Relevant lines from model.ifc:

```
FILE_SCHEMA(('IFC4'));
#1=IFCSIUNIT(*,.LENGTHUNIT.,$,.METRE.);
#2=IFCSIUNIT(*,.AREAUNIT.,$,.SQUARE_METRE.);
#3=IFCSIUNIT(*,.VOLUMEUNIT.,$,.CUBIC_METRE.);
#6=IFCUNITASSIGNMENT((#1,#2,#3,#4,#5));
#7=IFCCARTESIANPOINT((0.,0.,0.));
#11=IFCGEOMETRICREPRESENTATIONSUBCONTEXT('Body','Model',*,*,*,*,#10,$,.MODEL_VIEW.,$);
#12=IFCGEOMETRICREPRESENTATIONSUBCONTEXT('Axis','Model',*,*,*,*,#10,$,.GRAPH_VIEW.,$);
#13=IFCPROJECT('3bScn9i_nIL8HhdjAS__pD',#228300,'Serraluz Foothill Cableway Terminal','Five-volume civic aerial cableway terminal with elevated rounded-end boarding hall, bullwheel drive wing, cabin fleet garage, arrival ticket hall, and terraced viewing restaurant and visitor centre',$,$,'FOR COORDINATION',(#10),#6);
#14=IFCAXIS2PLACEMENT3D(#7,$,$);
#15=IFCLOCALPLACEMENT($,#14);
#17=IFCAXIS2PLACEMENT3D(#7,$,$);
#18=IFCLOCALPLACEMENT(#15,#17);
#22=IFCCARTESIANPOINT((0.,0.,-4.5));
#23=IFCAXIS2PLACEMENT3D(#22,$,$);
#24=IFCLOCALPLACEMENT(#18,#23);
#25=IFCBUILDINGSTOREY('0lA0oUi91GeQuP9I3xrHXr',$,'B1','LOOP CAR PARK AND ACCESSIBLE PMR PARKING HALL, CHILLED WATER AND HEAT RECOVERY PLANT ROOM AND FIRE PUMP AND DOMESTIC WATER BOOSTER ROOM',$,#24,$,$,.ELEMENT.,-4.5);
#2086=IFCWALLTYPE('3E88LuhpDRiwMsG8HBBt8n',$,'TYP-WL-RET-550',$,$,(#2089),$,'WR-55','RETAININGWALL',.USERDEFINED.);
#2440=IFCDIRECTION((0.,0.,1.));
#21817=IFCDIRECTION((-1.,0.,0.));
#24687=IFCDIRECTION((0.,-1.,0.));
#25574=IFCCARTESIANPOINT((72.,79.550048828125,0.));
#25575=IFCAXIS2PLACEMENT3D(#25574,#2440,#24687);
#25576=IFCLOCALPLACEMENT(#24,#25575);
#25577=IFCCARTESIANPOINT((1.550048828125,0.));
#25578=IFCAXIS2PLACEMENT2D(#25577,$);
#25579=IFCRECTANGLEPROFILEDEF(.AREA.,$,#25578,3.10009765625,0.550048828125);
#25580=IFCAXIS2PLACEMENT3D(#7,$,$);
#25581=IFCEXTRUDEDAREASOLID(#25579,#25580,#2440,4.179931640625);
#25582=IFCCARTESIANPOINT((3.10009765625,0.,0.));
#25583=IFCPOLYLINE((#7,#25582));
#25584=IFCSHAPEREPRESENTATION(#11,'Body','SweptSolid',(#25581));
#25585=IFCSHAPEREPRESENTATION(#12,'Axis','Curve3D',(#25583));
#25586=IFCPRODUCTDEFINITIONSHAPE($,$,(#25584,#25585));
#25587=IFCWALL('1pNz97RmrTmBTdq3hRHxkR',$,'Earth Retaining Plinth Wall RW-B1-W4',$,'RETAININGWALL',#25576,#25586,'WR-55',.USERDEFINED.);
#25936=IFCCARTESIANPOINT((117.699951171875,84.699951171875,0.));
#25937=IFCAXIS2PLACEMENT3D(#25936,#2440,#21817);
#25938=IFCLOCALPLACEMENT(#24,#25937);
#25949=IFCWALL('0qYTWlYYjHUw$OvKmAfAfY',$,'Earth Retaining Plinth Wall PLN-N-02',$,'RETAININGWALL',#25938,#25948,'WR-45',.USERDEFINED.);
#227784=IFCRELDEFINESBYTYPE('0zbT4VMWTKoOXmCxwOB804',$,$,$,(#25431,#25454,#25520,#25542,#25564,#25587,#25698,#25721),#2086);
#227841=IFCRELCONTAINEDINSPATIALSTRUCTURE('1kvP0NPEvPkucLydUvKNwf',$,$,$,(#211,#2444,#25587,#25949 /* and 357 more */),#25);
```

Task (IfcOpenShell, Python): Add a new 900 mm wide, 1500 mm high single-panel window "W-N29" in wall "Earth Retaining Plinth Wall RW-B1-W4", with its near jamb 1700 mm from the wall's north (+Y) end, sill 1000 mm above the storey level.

```python
import numpy as np
import ifcopenshell
import ifcopenshell.api.feature
import ifcopenshell.api.geometry
import ifcopenshell.api.root
import ifcopenshell.api.spatial
import ifcopenshell.geom
import ifcopenshell.util.element
import ifcopenshell.util.placement
import ifcopenshell.util.representation
import ifcopenshell.util.shape
import ifcopenshell.util.unit

model = ifcopenshell.open("model.ifc")
unit_scale = ifcopenshell.util.unit.calculate_unit_scale(model)
settings = ifcopenshell.geom.settings()


def volume(element):
    """Net volume in cubic metres, openings subtracted."""
    shape = ifcopenshell.geom.create_shape(settings, element)
    return ifcopenshell.util.shape.get_volume(shape.geometry)


wall = model.by_id(25587)
storey = ifcopenshell.util.element.get_container(wall, ifc_class="IfcBuildingStorey")
context = ifcopenshell.util.representation.get_context(model, "Model", "Body", "MODEL_VIEW")
before = volume(wall)

width, height, from_end, sill = 0.9, 1.5, 1.7, 1  # metres

# The wall runs along its own X axis, and the end named is its -X end.
wall_shape = ifcopenshell.geom.create_shape(settings, wall)
x, y, z = ifcopenshell.util.shape.get_vertices(wall_shape.geometry).T
start = x.min() + from_end
face, thickness = float(y.min()), float(y.max() - y.min())
wall_matrix = ifcopenshell.util.placement.get_local_placement(wall.ObjectPlacement)
level = ifcopenshell.util.placement.get_local_placement(storey.ObjectPlacement)[2, 3]


def in_wall(x, y):
    """Placement at x, y metres in the wall's axes, at sill height."""
    matrix = wall_matrix.copy()
    matrix[:, 3] = wall_matrix @ np.array([x / unit_scale, y / unit_scale, 0.0, 1.0])
    matrix[2, 3] = level + sill / unit_scale
    return matrix


# Opening: a box that overshoots both wall faces by 50 mm.
opening = ifcopenshell.api.root.create_entity(model, ifc_class="IfcOpeningElement", predefined_type="OPENING")
box = ifcopenshell.api.geometry.add_wall_representation(
    model, context=context, length=width, height=height, thickness=thickness + 0.1
)
ifcopenshell.api.geometry.assign_representation(model, product=opening, representation=box)
ifcopenshell.api.geometry.edit_object_placement(model, product=opening, matrix=in_wall(start, face - 0.05), is_si=False)
ifcopenshell.api.feature.add_feature(model, feature=opening, element=wall)

window = ifcopenshell.api.root.create_entity(model, ifc_class="IfcWindow", name="W-N29", predefined_type="WINDOW")
window.OverallWidth, window.OverallHeight = width / unit_scale, height / unit_scale
window.PartitioningType = "SINGLE_PANEL"
body = ifcopenshell.api.geometry.add_window_representation(
    model,
    context=context,
    overall_width=window.OverallWidth,
    overall_height=window.OverallHeight,
    partition_type="SINGLE_PANEL",
)
ifcopenshell.api.geometry.assign_representation(model, product=window, representation=body)
ifcopenshell.api.spatial.assign_container(model, products=[window], relating_structure=storey)
ifcopenshell.api.feature.add_filling(model, opening=opening, element=window)

# Centre the window in the wall's thickness.
ifcopenshell.api.geometry.edit_object_placement(model, product=window, matrix=in_wall(start, face), is_si=False)
window_shape = ifcopenshell.geom.create_shape(settings, window)
depth = ifcopenshell.util.shape.get_vertices(window_shape.geometry)[:, 1]
offset = face + thickness / 2 - (depth.min() + depth.max()) / 2
ifcopenshell.api.geometry.edit_object_placement(model, product=window, matrix=in_wall(start, offset), is_si=False)

after = volume(wall)

print(f"wall volume {before:.3f} -> {after:.3f} m3")

model.write("model_rev.ifc")
```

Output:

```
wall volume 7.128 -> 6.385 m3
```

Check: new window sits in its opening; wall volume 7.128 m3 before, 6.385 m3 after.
